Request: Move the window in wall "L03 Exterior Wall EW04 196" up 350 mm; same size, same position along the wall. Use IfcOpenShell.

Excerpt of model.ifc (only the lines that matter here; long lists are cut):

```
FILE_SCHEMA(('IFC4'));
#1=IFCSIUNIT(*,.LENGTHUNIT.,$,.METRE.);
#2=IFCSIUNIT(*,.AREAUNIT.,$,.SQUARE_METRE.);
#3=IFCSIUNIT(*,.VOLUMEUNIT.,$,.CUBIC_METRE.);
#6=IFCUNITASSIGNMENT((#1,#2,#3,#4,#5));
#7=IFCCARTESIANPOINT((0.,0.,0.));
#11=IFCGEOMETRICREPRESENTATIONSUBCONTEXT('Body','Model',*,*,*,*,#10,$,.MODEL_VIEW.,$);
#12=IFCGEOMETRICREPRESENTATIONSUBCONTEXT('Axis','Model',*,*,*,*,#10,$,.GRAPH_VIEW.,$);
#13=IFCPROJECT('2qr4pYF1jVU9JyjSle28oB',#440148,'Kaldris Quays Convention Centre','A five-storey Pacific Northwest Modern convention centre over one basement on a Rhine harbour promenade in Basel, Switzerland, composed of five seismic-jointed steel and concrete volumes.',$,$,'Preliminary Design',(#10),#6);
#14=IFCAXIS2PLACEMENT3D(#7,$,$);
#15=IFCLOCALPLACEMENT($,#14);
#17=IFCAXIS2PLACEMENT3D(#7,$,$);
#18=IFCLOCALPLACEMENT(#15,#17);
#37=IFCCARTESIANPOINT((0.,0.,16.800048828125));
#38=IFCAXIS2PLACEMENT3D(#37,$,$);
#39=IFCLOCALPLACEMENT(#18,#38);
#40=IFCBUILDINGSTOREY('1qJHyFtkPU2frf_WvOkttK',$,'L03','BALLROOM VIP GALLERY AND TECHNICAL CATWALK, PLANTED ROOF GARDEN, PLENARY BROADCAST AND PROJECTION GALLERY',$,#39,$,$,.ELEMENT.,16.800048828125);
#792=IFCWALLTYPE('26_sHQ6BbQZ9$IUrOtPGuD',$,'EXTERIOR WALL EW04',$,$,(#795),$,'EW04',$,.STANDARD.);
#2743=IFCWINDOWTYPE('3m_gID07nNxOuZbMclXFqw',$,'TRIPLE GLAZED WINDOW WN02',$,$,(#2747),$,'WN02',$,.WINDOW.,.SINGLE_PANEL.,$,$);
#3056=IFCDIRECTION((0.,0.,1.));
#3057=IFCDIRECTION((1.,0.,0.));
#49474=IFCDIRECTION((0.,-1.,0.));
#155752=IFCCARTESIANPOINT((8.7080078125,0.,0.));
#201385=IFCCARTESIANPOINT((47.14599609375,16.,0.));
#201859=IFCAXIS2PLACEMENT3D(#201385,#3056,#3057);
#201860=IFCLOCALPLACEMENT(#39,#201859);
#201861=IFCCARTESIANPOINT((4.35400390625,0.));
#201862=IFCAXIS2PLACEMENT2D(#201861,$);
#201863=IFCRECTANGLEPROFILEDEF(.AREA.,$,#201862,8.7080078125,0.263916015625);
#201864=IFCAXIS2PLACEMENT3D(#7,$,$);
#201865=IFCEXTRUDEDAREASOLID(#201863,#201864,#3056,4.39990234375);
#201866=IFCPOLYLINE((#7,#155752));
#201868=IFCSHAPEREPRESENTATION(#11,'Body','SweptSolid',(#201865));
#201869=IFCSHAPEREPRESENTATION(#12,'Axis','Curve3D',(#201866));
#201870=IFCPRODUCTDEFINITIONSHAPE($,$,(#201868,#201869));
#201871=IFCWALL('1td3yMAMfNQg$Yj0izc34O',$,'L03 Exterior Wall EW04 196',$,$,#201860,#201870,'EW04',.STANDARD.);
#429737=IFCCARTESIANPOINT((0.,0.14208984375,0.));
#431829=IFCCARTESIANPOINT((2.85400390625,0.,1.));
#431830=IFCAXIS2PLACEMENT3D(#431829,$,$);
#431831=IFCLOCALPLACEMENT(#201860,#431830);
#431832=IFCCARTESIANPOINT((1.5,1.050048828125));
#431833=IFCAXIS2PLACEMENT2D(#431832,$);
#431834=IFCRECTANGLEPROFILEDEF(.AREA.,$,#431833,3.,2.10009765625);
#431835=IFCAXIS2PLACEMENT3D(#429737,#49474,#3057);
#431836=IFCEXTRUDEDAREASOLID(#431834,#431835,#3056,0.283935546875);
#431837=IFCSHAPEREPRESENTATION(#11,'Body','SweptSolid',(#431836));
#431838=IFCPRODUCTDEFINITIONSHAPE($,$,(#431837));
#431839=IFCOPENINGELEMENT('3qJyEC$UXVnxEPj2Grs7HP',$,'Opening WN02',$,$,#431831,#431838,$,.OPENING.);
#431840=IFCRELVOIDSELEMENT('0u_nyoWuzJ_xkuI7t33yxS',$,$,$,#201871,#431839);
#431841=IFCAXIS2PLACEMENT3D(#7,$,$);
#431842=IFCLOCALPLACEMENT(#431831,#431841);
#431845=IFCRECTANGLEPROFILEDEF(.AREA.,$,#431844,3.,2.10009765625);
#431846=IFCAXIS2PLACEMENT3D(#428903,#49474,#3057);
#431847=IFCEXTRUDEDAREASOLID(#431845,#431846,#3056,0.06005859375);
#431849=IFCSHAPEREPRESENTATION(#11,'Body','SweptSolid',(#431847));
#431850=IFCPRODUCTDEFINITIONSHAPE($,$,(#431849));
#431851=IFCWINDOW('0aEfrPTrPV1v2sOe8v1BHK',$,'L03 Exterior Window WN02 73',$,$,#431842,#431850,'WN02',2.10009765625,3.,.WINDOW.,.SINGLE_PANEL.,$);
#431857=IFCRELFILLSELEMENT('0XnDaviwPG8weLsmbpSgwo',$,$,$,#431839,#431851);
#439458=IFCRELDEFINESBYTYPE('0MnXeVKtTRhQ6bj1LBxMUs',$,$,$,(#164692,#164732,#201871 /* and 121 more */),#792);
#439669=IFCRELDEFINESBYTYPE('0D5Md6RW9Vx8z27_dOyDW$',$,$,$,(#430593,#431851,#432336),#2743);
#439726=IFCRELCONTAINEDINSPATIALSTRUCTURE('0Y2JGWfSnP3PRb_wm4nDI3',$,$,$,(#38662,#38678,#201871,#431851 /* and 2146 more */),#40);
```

```python
import numpy as np
import ifcopenshell
import ifcopenshell.api.geometry
import ifcopenshell.util.placement
import ifcopenshell.util.unit

model = ifcopenshell.open("model.ifc")
unit_scale = ifcopenshell.util.unit.calculate_unit_scale(model)

window = model.by_guid("0aEfrPTrPV1v2sOe8v1BHK")
opening = window.FillsVoids[0].RelatingOpeningElement
dz = 0.35 / unit_scale

shift = np.array([0.0, 0.0, dz])
# The window is placed relative to its opening, so it follows when the opening moves.
matrix = ifcopenshell.util.placement.get_local_placement(opening.ObjectPlacement)
matrix[:3, 3] += shift
ifcopenshell.api.geometry.edit_object_placement(
    model, product=opening, matrix=matrix, is_si=False, should_transform_children=True
)

print(f"moved by {dz * unit_scale:+.3f} m")

model.write("model_v2.ifc")
```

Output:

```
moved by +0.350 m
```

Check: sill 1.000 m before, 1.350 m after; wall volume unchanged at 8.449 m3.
